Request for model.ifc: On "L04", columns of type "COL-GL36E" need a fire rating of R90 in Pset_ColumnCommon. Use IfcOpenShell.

First a look at what the model holds.

```python
import ifcopenshell
import ifcopenshell.util.element

model = ifcopenshell.open("model.ifc")
print(model.schema)
storey = next(s for s in model.by_type("IfcBuildingStorey") if s.Name == "L04")
columns = [e for e in ifcopenshell.util.element.get_decomposition(storey) if e.is_a("IfcColumn")]
seen = {}
for e in columns:
    element_type = ifcopenshell.util.element.get_type(e)
    key = (element_type.Name if element_type != e and element_type else None, ifcopenshell.util.element.get_pset(e, "Pset_ColumnCommon", "FireRating"))
    seen[key] = seen.get(key, 0) + 1
for (name, value), count in sorted(seen.items(), key=str):
    print(count, "x", name, "|", value)
```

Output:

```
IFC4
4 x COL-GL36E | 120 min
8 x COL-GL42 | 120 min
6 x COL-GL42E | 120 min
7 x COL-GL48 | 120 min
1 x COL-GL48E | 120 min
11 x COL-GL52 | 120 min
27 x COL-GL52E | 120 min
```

```python
import ifcopenshell
import ifcopenshell.api.pset
import ifcopenshell.util.element

model = ifcopenshell.open("model.ifc")

storey = next(s for s in model.by_type("IfcBuildingStorey") if s.Name == "L04")
columns = [e for e in ifcopenshell.util.element.get_decomposition(storey) if e.is_a("IfcColumn")]

count = 0
for e in columns:
    element_type = ifcopenshell.util.element.get_type(e)
    if element_type in (None, e) or element_type.Name != "COL-GL36E":
        continue
    # add_pset returns the element's existing set when there is one.
    pset = ifcopenshell.api.pset.add_pset(model, product=e, name="Pset_ColumnCommon")
    ifcopenshell.api.pset.edit_pset(model, pset=pset, properties={"FireRating": "R90"})
    count += 1

print(count, "columns updated")

model.write("model_edited.ifc")
```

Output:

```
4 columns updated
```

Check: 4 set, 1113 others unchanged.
